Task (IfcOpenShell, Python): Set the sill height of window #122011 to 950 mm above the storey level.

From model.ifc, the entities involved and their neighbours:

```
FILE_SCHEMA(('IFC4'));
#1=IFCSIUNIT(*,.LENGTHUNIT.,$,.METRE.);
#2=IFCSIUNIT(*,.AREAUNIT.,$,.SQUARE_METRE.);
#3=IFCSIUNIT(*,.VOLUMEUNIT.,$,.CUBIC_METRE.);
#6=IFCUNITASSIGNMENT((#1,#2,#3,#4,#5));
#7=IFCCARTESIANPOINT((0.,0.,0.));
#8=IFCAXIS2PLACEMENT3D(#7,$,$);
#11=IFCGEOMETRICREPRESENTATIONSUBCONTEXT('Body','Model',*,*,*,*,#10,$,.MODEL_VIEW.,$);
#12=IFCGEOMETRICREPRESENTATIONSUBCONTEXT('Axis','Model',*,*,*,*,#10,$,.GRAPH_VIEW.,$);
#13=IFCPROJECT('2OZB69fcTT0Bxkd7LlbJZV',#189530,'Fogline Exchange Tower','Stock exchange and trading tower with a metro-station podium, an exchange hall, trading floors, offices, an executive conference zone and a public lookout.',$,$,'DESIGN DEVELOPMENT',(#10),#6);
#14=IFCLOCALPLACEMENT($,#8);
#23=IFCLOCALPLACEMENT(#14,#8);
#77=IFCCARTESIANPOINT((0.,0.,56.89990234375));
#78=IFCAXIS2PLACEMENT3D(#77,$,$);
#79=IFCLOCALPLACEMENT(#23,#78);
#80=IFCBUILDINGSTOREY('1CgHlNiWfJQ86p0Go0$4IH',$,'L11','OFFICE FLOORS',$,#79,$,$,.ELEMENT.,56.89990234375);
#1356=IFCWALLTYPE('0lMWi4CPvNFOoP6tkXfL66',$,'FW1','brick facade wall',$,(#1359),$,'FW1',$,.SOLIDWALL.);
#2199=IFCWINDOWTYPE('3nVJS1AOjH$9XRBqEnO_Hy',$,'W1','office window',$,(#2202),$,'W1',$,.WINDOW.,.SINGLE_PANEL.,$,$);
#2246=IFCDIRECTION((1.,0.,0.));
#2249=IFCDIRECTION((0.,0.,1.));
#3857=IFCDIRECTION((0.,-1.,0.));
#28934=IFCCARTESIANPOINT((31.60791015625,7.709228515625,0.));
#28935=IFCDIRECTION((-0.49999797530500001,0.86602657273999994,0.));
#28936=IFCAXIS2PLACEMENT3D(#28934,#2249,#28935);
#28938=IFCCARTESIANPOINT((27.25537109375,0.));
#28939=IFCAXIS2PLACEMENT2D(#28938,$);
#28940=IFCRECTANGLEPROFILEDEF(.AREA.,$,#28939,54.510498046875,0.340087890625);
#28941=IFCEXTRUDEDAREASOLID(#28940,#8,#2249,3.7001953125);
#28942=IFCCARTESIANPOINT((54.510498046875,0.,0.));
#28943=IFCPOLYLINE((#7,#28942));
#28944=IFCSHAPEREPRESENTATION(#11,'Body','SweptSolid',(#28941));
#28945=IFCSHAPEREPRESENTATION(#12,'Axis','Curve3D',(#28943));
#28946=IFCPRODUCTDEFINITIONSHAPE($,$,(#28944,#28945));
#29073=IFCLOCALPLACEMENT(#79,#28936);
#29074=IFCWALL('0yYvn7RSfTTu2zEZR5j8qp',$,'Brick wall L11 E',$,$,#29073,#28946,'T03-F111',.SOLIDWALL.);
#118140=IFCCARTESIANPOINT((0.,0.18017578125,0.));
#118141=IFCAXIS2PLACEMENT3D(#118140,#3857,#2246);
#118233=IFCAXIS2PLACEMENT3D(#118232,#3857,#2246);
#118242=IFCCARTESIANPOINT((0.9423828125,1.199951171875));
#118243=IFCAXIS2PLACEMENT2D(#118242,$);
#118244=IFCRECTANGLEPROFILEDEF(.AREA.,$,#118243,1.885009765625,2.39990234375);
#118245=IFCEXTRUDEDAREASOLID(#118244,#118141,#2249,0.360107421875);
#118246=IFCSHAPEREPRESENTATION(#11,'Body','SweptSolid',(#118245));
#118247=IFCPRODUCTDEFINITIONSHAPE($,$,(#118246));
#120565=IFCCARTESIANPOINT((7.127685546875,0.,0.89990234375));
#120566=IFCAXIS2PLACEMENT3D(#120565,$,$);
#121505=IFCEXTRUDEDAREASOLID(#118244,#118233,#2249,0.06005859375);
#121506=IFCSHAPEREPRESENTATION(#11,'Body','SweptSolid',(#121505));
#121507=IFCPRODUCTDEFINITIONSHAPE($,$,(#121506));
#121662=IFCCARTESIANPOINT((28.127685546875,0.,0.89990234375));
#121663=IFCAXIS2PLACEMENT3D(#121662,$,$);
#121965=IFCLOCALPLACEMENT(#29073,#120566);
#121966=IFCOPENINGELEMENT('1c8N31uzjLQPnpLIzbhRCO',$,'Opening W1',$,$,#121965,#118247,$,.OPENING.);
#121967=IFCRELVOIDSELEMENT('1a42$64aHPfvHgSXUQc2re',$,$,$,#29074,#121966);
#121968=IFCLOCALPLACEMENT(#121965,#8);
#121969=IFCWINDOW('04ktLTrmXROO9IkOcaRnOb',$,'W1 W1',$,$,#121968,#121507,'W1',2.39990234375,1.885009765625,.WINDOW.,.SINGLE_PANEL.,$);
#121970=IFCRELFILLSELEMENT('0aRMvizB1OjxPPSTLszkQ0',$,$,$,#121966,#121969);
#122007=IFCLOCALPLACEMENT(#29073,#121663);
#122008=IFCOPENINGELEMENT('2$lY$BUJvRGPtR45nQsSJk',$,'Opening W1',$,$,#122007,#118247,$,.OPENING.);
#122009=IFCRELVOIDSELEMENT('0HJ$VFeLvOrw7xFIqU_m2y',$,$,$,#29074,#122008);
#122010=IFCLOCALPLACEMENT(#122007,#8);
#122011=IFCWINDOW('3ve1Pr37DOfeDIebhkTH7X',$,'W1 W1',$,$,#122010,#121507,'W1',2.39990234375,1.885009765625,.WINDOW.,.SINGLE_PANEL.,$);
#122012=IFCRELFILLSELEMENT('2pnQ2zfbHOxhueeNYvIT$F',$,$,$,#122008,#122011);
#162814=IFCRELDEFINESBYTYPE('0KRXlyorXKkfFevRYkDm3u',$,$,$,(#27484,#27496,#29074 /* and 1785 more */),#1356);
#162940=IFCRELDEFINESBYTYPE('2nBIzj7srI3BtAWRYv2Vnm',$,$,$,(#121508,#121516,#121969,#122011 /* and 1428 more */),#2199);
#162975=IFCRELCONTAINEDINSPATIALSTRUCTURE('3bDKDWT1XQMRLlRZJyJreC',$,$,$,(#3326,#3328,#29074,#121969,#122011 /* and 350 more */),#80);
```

```python
import numpy as np
import ifcopenshell
import ifcopenshell.api.geometry
import ifcopenshell.geom
import ifcopenshell.util.element
import ifcopenshell.util.placement
import ifcopenshell.util.shape
import ifcopenshell.util.unit

model = ifcopenshell.open("model.ifc")
unit_scale = ifcopenshell.util.unit.calculate_unit_scale(model)

window = model.by_guid("3ve1Pr37DOfeDIebhkTH7X")
opening = window.FillsVoids[0].RelatingOpeningElement
storey = ifcopenshell.util.element.get_container(window, ifc_class="IfcBuildingStorey")
level = ifcopenshell.util.placement.get_local_placement(storey.ObjectPlacement)[2, 3]

# The opening's origin need not be at the sill, so measure its lowest point.
shape = ifcopenshell.geom.create_shape(ifcopenshell.geom.settings(), opening)
bottom = ifcopenshell.util.shape.get_shape_bottom_elevation(shape, shape.geometry) / unit_scale
dz = level + 0.95 / unit_scale - bottom

shift = np.array([0.0, 0.0, dz])
# The window is placed relative to its opening, so it follows when the opening moves.
matrix = ifcopenshell.util.placement.get_local_placement(opening.ObjectPlacement)
matrix[:3, 3] += shift
ifcopenshell.api.geometry.edit_object_placement(
    model, product=opening, matrix=matrix, is_si=False, should_transform_children=True
)

print(f"moved by {dz * unit_scale:+.3f} m")

model.write("model_rev.ifc")
```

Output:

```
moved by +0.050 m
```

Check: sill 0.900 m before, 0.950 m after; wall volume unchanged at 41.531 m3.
